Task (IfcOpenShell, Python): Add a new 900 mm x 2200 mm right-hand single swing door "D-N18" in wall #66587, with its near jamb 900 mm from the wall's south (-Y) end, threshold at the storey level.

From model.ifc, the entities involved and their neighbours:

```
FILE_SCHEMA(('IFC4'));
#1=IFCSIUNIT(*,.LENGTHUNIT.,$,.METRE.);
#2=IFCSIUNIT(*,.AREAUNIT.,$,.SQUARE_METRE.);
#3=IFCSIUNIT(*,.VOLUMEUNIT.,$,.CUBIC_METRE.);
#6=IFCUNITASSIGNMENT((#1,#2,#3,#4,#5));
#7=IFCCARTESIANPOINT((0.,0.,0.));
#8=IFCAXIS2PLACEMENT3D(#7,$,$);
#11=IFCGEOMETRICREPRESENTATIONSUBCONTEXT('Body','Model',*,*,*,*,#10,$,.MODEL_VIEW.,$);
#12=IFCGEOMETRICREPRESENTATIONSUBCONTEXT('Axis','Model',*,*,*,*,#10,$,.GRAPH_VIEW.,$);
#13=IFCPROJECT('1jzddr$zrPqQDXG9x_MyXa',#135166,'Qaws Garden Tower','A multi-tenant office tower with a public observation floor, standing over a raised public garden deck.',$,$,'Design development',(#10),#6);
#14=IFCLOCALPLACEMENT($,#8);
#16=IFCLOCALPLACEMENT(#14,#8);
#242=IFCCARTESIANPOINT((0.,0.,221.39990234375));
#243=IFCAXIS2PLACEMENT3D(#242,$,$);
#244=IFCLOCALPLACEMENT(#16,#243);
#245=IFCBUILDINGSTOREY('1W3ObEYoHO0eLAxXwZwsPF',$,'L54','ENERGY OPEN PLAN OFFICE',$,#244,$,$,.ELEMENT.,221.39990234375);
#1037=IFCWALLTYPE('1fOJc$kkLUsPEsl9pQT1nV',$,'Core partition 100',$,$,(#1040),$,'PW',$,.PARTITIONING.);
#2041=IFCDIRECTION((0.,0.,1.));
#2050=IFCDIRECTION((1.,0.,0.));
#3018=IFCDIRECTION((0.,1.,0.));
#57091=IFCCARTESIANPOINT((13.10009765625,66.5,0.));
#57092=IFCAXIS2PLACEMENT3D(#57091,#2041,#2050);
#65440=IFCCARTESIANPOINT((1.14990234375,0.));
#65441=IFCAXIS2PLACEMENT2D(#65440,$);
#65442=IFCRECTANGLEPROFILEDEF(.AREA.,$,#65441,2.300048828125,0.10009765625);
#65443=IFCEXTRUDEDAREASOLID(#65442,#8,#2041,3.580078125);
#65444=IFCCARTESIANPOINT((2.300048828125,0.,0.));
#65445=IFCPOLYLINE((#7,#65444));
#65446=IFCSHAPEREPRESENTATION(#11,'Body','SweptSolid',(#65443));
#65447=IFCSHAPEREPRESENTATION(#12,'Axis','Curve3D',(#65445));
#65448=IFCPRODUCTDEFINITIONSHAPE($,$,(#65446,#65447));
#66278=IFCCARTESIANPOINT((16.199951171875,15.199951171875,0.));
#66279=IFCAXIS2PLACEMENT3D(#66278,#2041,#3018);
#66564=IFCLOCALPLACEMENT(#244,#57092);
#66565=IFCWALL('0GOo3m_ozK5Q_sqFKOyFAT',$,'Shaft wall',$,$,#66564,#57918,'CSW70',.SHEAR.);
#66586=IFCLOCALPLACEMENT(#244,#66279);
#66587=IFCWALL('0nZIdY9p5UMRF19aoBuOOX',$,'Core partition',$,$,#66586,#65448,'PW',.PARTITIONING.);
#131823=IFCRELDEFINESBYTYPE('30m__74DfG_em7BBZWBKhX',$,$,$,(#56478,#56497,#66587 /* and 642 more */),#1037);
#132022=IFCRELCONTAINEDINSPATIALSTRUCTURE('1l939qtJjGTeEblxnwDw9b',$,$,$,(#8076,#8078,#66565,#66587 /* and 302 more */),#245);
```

```python
import numpy as np
import ifcopenshell
import ifcopenshell.api.feature
import ifcopenshell.api.geometry
import ifcopenshell.api.root
import ifcopenshell.api.spatial
import ifcopenshell.geom
import ifcopenshell.util.element
import ifcopenshell.util.placement
import ifcopenshell.util.representation
import ifcopenshell.util.shape
import ifcopenshell.util.unit

model = ifcopenshell.open("model.ifc")
unit_scale = ifcopenshell.util.unit.calculate_unit_scale(model)
settings = ifcopenshell.geom.settings()


def volume(element):
    """Net volume in cubic metres, openings subtracted."""
    shape = ifcopenshell.geom.create_shape(settings, element)
    return ifcopenshell.util.shape.get_volume(shape.geometry)


wall = model.by_guid("0nZIdY9p5UMRF19aoBuOOX")
storey = ifcopenshell.util.element.get_container(wall, ifc_class="IfcBuildingStorey")
context = ifcopenshell.util.representation.get_context(model, "Model", "Body", "MODEL_VIEW")
before = volume(wall)

width, height, from_end, sill = 0.9, 2.2, 0.9, 0.0  # metres

# The wall runs along its own X axis, and the end named is its -X end.
wall_shape = ifcopenshell.geom.create_shape(settings, wall)
x, y, z = ifcopenshell.util.shape.get_vertices(wall_shape.geometry).T
start = x.min() + from_end
face, thickness = float(y.min()), float(y.max() - y.min())
wall_matrix = ifcopenshell.util.placement.get_local_placement(wall.ObjectPlacement)
level = ifcopenshell.util.placement.get_local_placement(storey.ObjectPlacement)[2, 3]


def in_wall(x, y):
    """Placement at x, y metres in the wall's axes, at sill height."""
    matrix = wall_matrix.copy()
    matrix[:, 3] = wall_matrix @ np.array([x / unit_scale, y / unit_scale, 0.0, 1.0])
    matrix[2, 3] = level + sill / unit_scale
    return matrix


# Opening: a box that overshoots both wall faces by 50 mm.
opening = ifcopenshell.api.root.create_entity(model, ifc_class="IfcOpeningElement", predefined_type="OPENING")
box = ifcopenshell.api.geometry.add_wall_representation(
    model, context=context, length=width, height=height, thickness=thickness + 0.1
)
ifcopenshell.api.geometry.assign_representation(model, product=opening, representation=box)
ifcopenshell.api.geometry.edit_object_placement(model, product=opening, matrix=in_wall(start, face - 0.05), is_si=False)
ifcopenshell.api.feature.add_feature(model, feature=opening, element=wall)

door = ifcopenshell.api.root.create_entity(model, ifc_class="IfcDoor", name="D-N18", predefined_type="DOOR")
door.OverallWidth, door.OverallHeight = width / unit_scale, height / unit_scale
door.OperationType = "SINGLE_SWING_RIGHT"
body = ifcopenshell.api.geometry.add_door_representation(
    model,
    context=context,
    overall_width=door.OverallWidth,
    overall_height=door.OverallHeight,
    operation_type="SINGLE_SWING_RIGHT",
    lining_properties={"LiningDepth": thickness / unit_scale, "ThresholdDepth": thickness / unit_scale},
)
ifcopenshell.api.geometry.assign_representation(model, product=door, representation=body)
ifcopenshell.api.spatial.assign_container(model, products=[door], relating_structure=storey)
ifcopenshell.api.feature.add_filling(model, opening=opening, element=door)

# The lining spans the wall, so the door starts at the wall face.
ifcopenshell.api.geometry.edit_object_placement(model, product=door, matrix=in_wall(start, face), is_si=False)

after = volume(wall)

print(f"wall volume {before:.3f} -> {after:.3f} m3")

model.write("model_rev.ifc")
```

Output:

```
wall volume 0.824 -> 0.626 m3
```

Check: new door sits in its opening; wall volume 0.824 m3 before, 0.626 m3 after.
